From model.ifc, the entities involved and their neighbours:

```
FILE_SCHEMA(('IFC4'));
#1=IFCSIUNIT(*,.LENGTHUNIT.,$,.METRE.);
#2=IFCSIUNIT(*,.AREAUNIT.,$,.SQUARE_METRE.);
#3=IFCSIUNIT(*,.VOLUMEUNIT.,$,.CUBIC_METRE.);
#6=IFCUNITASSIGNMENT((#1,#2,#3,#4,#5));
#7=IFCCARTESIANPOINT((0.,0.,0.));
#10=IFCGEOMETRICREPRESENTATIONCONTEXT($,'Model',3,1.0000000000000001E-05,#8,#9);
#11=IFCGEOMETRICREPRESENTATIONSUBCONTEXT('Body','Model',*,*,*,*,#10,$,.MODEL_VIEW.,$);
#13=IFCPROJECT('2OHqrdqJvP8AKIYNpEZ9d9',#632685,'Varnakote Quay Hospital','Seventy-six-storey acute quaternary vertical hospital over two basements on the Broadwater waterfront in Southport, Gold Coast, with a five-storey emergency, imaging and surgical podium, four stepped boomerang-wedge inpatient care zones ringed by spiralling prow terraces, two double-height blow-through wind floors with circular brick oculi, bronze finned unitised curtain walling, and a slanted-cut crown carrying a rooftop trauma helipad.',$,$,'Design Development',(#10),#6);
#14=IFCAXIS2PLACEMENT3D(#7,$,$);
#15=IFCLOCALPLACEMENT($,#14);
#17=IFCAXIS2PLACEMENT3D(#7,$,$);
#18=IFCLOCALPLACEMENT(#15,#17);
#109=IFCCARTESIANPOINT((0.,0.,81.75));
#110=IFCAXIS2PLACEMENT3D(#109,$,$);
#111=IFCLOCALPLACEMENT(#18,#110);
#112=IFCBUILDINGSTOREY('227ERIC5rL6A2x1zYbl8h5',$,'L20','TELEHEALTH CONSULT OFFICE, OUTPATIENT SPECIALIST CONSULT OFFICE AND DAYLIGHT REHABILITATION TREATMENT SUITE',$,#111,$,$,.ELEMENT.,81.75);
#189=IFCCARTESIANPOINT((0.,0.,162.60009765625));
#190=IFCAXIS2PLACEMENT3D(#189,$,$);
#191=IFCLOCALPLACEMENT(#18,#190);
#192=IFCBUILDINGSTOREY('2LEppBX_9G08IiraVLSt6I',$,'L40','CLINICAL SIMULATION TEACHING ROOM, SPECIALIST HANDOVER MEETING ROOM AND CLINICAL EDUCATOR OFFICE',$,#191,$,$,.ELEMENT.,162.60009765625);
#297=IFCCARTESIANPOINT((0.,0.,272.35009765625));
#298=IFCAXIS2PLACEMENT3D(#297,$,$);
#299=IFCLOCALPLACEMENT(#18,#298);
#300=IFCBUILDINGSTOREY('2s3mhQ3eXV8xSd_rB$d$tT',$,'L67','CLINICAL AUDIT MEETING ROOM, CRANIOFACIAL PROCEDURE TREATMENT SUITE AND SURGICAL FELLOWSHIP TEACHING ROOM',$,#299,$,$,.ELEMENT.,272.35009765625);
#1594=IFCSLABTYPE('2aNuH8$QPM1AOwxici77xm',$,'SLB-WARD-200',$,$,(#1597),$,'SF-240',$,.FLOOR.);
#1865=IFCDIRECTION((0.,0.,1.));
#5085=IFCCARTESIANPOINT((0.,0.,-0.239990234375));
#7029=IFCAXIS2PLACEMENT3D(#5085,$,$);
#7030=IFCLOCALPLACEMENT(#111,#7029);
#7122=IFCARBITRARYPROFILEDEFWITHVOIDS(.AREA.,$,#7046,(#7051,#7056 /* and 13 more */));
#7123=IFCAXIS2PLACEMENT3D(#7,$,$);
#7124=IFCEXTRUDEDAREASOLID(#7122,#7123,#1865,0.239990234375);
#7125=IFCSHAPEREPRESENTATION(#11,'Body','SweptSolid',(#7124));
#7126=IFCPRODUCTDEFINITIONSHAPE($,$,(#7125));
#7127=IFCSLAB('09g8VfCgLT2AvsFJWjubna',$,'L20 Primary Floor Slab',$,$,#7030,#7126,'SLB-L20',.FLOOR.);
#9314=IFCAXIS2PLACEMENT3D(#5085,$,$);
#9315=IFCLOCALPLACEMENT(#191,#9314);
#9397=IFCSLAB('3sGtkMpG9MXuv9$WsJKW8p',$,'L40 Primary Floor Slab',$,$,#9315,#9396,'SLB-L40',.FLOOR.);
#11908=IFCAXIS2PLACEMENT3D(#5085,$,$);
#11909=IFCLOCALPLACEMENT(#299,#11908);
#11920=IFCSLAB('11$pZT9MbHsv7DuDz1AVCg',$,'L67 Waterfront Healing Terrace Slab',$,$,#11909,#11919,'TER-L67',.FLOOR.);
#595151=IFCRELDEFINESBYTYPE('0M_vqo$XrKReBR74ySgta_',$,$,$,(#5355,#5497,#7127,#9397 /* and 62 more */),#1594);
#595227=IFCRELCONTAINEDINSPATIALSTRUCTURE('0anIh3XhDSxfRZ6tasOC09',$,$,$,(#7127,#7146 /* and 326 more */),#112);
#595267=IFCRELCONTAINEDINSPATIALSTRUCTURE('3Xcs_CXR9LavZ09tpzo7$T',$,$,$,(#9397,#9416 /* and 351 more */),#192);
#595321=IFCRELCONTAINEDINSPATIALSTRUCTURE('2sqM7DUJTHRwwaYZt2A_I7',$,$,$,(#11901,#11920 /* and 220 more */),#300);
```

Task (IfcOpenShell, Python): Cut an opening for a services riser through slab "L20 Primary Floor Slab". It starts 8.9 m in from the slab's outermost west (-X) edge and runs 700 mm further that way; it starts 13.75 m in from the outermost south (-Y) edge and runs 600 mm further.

```python
import numpy as np
import ifcopenshell
import ifcopenshell.api.feature
import ifcopenshell.api.geometry
import ifcopenshell.api.root
import ifcopenshell.geom
import ifcopenshell.util.placement
import ifcopenshell.util.representation
import ifcopenshell.util.shape
import ifcopenshell.util.unit

model = ifcopenshell.open("model.ifc")
unit_scale = ifcopenshell.util.unit.calculate_unit_scale(model)
settings = ifcopenshell.geom.settings()


def volume(element):
    """Net volume in cubic metres, openings subtracted."""
    shape = ifcopenshell.geom.create_shape(settings, element)
    return ifcopenshell.util.shape.get_volume(shape.geometry)


slab = model.by_id(7127)
before = volume(slab)

# Extent in the slab's own axes, in metres. The edges named are its -X and -Y sides.
slab_shape = ifcopenshell.geom.create_shape(settings, slab)
vertices = ifcopenshell.util.shape.get_vertices(slab_shape.geometry)
x_min, y_min, bottom = vertices.min(axis=0)
top = vertices[:, 2].max()

opening = ifcopenshell.api.root.create_entity(model, ifc_class="IfcOpeningElement", name="Services riser opening", predefined_type="OPENING")
context = ifcopenshell.util.representation.get_context(model, "Model", "Body", "MODEL_VIEW")
width, depth = 0.7, 0.6
outline = [(0.0, 0.0), (width, 0.0), (width, depth), (0.0, depth), (0.0, 0.0)]
# Overshoot both faces by 50 mm so the cut is clean.
shape = ifcopenshell.api.geometry.add_slab_representation(
    model, context=context, depth=top - bottom + 0.1, polyline=outline
)
ifcopenshell.api.geometry.assign_representation(model, product=opening, representation=shape)

matrix = ifcopenshell.util.placement.get_local_placement(slab.ObjectPlacement)
matrix[:, 3] = matrix @ np.append(np.array([x_min + 8.9, y_min + 13.75, bottom - 0.05]) / unit_scale, 1.0)
ifcopenshell.api.geometry.edit_object_placement(model, product=opening, matrix=matrix, is_si=False)
ifcopenshell.api.feature.add_feature(model, feature=opening, element=slab)

after = volume(slab)

print(f"slab volume {before:.3f} -> {after:.3f} m3")

model.write("model_v2.ifc")
```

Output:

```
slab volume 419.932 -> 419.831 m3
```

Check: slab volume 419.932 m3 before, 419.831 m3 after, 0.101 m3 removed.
